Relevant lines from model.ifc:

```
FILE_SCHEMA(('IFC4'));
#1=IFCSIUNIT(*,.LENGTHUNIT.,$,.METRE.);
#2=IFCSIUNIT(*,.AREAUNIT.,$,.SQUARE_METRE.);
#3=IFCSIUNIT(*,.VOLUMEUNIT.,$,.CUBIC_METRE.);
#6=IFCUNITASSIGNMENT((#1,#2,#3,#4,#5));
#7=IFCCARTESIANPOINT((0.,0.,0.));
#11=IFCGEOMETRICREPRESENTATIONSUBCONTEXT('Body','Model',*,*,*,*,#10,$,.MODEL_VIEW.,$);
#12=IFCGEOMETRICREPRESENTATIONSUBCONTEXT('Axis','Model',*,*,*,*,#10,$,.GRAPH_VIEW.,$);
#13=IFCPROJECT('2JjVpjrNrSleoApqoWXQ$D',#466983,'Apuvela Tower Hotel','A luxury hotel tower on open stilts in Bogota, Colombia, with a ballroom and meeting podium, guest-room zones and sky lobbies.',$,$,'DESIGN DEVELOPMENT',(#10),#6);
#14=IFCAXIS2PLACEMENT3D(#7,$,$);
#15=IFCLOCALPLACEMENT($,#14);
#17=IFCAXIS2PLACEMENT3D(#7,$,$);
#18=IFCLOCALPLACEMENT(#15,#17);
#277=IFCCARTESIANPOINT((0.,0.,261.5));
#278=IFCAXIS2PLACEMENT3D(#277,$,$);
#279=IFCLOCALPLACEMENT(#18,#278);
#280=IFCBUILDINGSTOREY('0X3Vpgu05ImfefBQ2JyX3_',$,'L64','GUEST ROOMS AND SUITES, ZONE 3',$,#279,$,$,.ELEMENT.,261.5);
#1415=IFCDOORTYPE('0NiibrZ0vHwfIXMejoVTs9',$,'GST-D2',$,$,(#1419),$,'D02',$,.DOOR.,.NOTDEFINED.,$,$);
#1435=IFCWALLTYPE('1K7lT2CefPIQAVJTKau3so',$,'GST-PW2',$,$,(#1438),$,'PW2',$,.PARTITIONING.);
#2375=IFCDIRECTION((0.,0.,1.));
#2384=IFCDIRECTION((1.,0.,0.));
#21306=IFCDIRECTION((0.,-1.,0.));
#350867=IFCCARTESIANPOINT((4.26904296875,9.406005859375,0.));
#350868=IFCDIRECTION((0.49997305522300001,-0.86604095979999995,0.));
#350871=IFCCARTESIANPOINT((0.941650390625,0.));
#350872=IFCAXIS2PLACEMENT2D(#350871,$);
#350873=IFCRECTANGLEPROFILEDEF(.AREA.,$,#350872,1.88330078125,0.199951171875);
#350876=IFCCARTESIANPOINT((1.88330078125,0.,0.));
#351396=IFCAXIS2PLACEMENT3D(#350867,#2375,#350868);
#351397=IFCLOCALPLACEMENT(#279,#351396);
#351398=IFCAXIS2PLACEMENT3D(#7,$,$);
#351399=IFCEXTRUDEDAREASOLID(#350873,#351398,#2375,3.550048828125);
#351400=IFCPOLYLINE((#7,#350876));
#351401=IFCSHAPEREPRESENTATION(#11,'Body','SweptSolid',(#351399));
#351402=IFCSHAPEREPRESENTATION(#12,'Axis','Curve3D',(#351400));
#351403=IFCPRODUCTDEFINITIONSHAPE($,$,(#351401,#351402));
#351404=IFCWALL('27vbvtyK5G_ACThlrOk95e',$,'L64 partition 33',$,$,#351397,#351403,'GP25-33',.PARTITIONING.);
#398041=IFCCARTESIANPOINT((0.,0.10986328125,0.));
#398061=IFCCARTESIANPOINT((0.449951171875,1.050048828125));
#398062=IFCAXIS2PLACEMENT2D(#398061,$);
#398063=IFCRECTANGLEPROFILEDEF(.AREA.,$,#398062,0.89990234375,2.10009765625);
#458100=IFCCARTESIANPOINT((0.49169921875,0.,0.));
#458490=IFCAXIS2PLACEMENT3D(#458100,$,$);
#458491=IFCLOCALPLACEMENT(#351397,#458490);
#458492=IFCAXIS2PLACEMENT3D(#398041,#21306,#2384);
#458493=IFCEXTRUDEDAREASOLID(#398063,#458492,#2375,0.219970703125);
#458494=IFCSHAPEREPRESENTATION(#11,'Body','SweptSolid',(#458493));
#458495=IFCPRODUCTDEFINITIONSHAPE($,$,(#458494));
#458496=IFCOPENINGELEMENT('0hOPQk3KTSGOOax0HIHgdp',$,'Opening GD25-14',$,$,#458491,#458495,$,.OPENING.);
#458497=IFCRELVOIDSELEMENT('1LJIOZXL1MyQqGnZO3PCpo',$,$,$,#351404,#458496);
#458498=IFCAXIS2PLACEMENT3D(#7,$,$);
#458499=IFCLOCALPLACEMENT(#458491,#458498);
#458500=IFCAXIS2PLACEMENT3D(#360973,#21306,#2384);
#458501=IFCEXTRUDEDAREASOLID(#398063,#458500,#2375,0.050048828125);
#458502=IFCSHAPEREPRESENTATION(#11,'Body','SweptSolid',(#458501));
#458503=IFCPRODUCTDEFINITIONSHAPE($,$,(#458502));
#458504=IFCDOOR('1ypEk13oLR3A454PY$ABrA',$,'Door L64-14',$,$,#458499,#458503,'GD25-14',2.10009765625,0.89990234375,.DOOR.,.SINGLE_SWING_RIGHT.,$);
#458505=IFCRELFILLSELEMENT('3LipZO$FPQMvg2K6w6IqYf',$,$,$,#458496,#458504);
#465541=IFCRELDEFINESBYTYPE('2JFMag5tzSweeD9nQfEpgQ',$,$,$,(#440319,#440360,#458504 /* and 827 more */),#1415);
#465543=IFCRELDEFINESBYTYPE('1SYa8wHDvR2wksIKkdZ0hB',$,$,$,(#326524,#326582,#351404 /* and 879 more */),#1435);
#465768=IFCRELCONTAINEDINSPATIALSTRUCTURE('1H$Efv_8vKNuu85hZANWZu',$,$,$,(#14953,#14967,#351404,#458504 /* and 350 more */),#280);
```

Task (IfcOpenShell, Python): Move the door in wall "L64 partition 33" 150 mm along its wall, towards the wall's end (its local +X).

```python
import ifcopenshell
import ifcopenshell.api.geometry
import ifcopenshell.util.placement
import ifcopenshell.util.unit

model = ifcopenshell.open("model.ifc")
unit_scale = ifcopenshell.util.unit.calculate_unit_scale(model)

door = model.by_guid("1ypEk13oLR3A454PY$ABrA")
opening = door.FillsVoids[0].RelatingOpeningElement
wall = opening.VoidsElements[0].RelatingBuildingElement

wall_matrix = ifcopenshell.util.placement.get_local_placement(wall.ObjectPlacement)
shift = wall_matrix[:3, 0] * 0.15 / unit_scale
before = ifcopenshell.util.placement.get_local_placement(door.ObjectPlacement)[:3, 3].copy()

# The door is placed relative to its opening, so it follows when the opening moves.
matrix = ifcopenshell.util.placement.get_local_placement(opening.ObjectPlacement)
matrix[:3, 3] += shift
ifcopenshell.api.geometry.edit_object_placement(
    model, product=opening, matrix=matrix, is_si=False, should_transform_children=True
)

after = ifcopenshell.util.placement.get_local_placement(door.ObjectPlacement)[:3, 3]
print("door moved by", (after - before).round(3) + 0.0)

model.write("model-out.ifc")
```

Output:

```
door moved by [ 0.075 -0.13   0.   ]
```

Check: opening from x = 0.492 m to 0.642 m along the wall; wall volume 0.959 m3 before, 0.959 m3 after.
